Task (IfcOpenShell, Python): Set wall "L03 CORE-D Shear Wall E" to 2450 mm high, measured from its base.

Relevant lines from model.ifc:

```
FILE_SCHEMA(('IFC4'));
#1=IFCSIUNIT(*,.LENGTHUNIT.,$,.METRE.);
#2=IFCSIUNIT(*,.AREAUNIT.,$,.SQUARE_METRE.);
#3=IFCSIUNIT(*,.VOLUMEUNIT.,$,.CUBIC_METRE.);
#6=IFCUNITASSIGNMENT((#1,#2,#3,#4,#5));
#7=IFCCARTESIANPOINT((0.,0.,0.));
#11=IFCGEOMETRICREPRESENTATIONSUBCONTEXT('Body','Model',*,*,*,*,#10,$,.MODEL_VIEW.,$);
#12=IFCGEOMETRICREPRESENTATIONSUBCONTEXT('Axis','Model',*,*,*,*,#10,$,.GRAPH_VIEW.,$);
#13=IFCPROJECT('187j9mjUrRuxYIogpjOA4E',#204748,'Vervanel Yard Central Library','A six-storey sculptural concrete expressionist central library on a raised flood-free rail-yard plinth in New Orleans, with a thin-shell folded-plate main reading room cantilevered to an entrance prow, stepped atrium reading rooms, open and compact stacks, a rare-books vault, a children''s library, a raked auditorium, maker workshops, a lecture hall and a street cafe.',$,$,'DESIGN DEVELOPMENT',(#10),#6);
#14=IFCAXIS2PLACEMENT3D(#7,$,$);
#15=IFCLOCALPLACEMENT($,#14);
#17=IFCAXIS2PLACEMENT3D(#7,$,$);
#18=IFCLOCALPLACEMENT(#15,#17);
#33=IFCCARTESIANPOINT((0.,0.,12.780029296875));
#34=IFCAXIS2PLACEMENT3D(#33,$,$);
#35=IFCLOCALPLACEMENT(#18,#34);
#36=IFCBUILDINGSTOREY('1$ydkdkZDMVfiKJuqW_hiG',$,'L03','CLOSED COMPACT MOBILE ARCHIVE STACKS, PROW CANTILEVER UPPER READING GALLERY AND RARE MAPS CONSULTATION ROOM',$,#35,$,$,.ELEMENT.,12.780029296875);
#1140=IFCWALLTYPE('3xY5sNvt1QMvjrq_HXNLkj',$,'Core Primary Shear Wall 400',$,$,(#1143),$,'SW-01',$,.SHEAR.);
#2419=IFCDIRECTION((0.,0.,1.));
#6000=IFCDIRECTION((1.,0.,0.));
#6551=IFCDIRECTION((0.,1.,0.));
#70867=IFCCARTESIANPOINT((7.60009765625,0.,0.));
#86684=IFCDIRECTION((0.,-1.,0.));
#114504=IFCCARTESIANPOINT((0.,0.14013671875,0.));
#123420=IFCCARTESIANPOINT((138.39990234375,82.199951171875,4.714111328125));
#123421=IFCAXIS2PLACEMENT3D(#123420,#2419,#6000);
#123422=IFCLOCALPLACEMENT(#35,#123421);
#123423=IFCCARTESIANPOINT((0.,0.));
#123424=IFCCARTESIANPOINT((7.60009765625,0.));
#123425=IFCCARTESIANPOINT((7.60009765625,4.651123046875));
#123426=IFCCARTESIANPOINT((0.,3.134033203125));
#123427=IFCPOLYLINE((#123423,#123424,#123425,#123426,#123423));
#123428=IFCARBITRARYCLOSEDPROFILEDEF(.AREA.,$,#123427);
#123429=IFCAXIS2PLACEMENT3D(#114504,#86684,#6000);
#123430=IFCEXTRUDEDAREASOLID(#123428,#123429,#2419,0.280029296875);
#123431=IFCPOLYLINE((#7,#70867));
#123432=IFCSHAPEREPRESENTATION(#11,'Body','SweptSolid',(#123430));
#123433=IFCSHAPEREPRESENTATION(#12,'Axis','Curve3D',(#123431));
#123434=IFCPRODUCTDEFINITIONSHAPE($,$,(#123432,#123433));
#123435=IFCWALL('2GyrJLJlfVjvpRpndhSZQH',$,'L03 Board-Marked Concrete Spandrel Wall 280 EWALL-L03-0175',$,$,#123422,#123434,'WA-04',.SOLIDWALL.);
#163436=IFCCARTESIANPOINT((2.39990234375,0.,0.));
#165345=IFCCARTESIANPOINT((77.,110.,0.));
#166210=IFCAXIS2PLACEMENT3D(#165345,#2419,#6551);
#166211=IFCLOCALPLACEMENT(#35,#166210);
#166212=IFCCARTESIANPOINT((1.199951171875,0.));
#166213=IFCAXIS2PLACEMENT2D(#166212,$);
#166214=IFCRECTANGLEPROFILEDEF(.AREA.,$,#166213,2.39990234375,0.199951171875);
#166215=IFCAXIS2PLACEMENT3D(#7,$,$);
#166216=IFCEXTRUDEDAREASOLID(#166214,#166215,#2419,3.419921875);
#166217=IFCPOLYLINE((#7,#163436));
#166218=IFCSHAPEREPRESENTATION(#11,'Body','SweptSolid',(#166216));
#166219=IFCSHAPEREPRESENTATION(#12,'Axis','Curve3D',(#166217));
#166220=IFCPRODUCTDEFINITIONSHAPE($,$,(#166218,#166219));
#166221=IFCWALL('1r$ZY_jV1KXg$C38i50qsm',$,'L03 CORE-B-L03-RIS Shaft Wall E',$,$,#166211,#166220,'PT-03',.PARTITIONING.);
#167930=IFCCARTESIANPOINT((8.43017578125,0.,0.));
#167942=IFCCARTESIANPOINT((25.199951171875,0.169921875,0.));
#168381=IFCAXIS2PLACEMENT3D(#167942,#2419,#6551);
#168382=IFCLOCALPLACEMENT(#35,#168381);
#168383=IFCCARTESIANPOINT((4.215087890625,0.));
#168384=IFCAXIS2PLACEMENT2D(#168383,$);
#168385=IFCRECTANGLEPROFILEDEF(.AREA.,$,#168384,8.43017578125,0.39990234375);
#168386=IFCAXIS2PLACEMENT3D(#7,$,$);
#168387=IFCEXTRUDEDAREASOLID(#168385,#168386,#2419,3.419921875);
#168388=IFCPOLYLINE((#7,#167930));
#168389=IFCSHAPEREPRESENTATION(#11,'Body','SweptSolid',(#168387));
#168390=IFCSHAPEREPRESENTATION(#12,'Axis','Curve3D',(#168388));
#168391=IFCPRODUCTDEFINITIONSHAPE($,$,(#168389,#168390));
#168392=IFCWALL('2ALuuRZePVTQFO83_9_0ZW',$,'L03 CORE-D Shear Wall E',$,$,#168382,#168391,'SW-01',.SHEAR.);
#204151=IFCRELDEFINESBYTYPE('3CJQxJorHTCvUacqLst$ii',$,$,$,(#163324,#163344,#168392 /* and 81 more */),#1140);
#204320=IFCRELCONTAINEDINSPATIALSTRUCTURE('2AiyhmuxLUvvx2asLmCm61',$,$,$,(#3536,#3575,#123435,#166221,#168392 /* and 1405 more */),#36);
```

```python
import ifcopenshell
import ifcopenshell.geom
import ifcopenshell.util.representation
import ifcopenshell.util.shape
import ifcopenshell.util.unit

model = ifcopenshell.open("model.ifc")
unit_scale = ifcopenshell.util.unit.calculate_unit_scale(model)
settings = ifcopenshell.geom.settings()


def volume(element):
    """Net volume in cubic metres, openings subtracted."""
    shape = ifcopenshell.geom.create_shape(settings, element)
    return ifcopenshell.util.shape.get_volume(shape.geometry)


wall = model.by_guid("2ALuuRZePVTQFO83_9_0ZW")
before = volume(wall)

body = ifcopenshell.util.representation.get_representation(wall, "Model", "Body")
solid = body.Items[0]
old_height = solid.Depth
solid.Depth = 2.45 / unit_scale
after = volume(wall)

print(f"height {old_height:g} -> {solid.Depth:g}, volume {before:.3f} -> {after:.3f} m3")

model.write("model_rev.ifc")
```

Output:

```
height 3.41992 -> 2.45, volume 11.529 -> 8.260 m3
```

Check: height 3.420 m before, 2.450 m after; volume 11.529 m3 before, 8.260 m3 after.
